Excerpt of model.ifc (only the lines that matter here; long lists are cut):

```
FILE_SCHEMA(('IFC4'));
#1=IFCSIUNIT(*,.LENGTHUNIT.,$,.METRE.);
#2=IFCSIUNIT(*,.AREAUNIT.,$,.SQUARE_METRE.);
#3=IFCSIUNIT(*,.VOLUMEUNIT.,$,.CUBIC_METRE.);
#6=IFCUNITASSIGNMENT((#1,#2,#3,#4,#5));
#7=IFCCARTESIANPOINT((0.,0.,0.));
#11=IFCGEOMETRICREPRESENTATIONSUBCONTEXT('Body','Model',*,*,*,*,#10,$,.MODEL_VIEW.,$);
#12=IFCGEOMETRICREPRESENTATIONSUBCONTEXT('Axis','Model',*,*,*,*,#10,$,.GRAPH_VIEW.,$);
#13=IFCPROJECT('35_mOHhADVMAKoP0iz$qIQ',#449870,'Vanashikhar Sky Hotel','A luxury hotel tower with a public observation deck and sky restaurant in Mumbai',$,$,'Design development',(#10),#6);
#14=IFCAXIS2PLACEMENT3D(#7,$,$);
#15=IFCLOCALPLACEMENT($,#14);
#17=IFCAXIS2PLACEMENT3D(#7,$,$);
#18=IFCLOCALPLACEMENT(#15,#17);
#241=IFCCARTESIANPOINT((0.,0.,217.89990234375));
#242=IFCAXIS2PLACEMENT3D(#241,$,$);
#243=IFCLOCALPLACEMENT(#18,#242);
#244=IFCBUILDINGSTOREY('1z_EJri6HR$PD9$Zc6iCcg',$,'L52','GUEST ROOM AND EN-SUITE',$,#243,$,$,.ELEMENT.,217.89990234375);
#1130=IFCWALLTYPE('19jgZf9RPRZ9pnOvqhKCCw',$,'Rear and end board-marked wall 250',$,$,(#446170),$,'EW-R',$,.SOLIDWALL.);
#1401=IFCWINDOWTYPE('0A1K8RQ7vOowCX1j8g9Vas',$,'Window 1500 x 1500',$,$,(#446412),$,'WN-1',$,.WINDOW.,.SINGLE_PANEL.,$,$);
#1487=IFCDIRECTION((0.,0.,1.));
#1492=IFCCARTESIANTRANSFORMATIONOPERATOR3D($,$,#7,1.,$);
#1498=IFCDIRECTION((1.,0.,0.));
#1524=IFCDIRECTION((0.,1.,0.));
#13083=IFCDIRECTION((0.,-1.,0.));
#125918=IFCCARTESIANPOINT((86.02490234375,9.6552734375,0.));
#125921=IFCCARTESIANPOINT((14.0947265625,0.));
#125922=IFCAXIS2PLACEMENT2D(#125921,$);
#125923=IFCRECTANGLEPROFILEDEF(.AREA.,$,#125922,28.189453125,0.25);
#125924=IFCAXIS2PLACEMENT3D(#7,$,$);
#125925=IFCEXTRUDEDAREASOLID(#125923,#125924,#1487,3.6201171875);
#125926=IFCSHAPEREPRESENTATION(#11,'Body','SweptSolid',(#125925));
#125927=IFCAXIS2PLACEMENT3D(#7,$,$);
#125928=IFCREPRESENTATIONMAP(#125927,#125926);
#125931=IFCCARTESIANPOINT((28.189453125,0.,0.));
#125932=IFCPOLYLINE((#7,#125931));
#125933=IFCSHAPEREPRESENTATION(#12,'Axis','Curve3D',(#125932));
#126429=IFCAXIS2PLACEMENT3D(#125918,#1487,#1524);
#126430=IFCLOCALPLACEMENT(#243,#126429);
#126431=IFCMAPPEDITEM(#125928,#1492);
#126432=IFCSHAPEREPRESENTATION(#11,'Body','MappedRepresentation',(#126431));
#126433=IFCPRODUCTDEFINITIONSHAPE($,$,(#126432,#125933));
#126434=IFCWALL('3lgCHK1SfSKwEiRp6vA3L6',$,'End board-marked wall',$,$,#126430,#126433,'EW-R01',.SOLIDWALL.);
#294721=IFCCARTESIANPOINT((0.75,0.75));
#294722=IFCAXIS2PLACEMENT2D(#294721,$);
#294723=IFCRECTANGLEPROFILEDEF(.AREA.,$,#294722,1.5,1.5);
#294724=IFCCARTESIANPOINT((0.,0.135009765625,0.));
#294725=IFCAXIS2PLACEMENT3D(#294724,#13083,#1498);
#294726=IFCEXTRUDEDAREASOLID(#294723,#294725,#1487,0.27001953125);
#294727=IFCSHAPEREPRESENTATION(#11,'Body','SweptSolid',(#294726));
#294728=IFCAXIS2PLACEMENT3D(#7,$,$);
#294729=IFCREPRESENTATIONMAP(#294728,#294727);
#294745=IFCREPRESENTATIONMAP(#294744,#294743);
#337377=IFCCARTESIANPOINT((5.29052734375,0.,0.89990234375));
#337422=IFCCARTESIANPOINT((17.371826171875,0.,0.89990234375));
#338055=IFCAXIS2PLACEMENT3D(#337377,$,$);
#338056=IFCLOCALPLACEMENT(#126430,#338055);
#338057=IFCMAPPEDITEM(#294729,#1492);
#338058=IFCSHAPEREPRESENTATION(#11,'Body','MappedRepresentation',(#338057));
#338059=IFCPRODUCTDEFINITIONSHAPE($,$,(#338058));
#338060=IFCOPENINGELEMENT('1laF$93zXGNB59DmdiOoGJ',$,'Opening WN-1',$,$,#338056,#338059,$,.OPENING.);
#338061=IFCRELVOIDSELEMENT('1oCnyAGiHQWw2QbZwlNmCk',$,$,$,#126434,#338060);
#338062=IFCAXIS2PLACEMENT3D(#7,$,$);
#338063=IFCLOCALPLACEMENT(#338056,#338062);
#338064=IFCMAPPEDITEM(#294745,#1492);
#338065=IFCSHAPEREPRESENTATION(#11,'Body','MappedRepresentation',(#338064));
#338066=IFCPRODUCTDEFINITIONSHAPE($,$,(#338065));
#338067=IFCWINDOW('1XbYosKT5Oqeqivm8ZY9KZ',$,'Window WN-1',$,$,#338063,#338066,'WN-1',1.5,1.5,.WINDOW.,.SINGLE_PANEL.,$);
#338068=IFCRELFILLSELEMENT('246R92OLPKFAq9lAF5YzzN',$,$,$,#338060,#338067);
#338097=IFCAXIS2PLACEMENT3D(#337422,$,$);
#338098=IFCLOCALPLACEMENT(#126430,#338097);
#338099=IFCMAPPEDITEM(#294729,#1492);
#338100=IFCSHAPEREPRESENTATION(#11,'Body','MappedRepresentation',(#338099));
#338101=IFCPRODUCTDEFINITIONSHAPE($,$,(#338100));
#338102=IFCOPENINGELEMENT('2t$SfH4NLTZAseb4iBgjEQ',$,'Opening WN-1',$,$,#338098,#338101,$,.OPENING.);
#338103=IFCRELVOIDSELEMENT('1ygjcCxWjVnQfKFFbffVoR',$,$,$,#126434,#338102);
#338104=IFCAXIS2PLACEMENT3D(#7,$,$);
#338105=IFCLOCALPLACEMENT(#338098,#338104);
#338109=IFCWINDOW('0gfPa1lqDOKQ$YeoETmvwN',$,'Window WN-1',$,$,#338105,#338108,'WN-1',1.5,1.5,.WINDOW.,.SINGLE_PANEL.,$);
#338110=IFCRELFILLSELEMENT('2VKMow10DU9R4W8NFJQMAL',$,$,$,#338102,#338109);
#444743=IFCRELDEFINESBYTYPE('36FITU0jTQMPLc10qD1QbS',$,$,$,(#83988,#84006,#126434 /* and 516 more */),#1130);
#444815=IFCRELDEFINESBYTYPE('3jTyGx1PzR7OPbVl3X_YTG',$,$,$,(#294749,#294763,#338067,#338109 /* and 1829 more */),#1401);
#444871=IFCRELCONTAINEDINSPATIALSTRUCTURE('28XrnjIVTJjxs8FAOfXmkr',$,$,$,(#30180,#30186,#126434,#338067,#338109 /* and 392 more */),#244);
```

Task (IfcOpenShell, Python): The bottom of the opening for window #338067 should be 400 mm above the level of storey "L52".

```python
import numpy as np
import ifcopenshell
import ifcopenshell.api.geometry
import ifcopenshell.geom
import ifcopenshell.util.element
import ifcopenshell.util.placement
import ifcopenshell.util.shape
import ifcopenshell.util.unit

model = ifcopenshell.open("model.ifc")
unit_scale = ifcopenshell.util.unit.calculate_unit_scale(model)

window = model.by_guid("1XbYosKT5Oqeqivm8ZY9KZ")
opening = window.FillsVoids[0].RelatingOpeningElement
storey = ifcopenshell.util.element.get_container(window, ifc_class="IfcBuildingStorey")
level = ifcopenshell.util.placement.get_local_placement(storey.ObjectPlacement)[2, 3]

# The opening's origin need not be at the sill, so measure its lowest point.
shape = ifcopenshell.geom.create_shape(ifcopenshell.geom.settings(), opening)
bottom = ifcopenshell.util.shape.get_shape_bottom_elevation(shape, shape.geometry) / unit_scale
dz = level + 0.4 - bottom

shift = np.array([0.0, 0.0, dz])
# The window is placed relative to its opening, so it follows when the opening moves.
matrix = ifcopenshell.util.placement.get_local_placement(opening.ObjectPlacement)
matrix[:3, 3] += shift
ifcopenshell.api.geometry.edit_object_placement(
    model, product=opening, matrix=matrix, is_si=False, should_transform_children=True
)

print(f"moved by {dz * unit_scale:+.3f} m")

model.write("model_updated.ifc")
```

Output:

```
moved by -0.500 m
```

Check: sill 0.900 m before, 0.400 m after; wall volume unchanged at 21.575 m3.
